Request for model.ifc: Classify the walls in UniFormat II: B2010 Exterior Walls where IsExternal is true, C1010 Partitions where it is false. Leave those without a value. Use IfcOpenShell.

First a look at what the model holds.

```python
import ifcopenshell
import ifcopenshell.util.element

model = ifcopenshell.open("model.ifc")
print(model.schema)
print("classifications:", [c.Name for c in model.by_type("IfcClassification")])
values = [ifcopenshell.util.element.get_pset(e, "Pset_WallCommon", "IsExternal") for e in model.by_type("IfcWall")]
for value in (True, False, None):
    print("IsExternal", value, values.count(value))
```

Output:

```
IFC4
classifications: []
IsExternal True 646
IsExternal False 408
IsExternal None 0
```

```python
import ifcopenshell
import ifcopenshell.api.classification
import ifcopenshell.util.element

model = ifcopenshell.open("model.ifc")

system = ifcopenshell.api.classification.add_classification(model, classification="UniFormat II")

walls = model.by_type("IfcWall")
external = {e: ifcopenshell.util.element.get_pset(e, "Pset_WallCommon", "IsExternal") for e in walls}
for flag, code, name in ((True, "B2010", "Exterior Walls"), (False, "C1010", "Partitions")):
    products = [e for e in walls if external[e] is flag]
    ifcopenshell.api.classification.add_reference(
        model, products=products, classification=system, identification=code, name=name
    )
    print(code, len(products))

model.write("model_edited.ifc")
```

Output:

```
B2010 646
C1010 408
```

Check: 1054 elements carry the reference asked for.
